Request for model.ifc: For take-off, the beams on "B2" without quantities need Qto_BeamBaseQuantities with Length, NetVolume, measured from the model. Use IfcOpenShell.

First a look at what the model holds.

```python
import ifcopenshell
import ifcopenshell.util.element
import ifcopenshell.util.unit

model = ifcopenshell.open("model.ifc")
print(model.schema)
for unit_type in ("LENGTHUNIT", "AREAUNIT", "VOLUMEUNIT"):
    print(unit_type, ifcopenshell.util.unit.calculate_unit_scale(model, unit_type))
storey = next(s for s in model.by_type("IfcBuildingStorey") if s.Name == "B2")
beams = [e for e in ifcopenshell.util.element.get_decomposition(storey) if e.is_a("IfcBeam")]
for e in sorted(beams, key=lambda e: e.id()):
    print(e.id(), e.is_a(), e.Name, list(ifcopenshell.util.element.get_psets(e, qtos_only=True)), sep=" | ")
```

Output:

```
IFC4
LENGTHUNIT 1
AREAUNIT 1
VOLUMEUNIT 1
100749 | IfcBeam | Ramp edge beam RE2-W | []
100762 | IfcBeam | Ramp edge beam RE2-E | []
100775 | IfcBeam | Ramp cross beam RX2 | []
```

```python
import ifcopenshell
import ifcopenshell.api.pset
import ifcopenshell.geom
import ifcopenshell.util.element
import ifcopenshell.util.shape
import ifcopenshell.util.unit

model = ifcopenshell.open("model.ifc")
unit_scale = ifcopenshell.util.unit.calculate_unit_scale(model)
volume_scale = ifcopenshell.util.unit.calculate_unit_scale(model, "VOLUMEUNIT")
settings = ifcopenshell.geom.settings()

storey = next(s for s in model.by_type("IfcBuildingStorey") if s.Name == "B2")
beams = [e for e in ifcopenshell.util.element.get_decomposition(storey) if e.is_a("IfcBeam")]

for e in sorted(beams, key=lambda e: e.id()):
    if ifcopenshell.util.element.get_psets(e, qtos_only=True, should_inherit=False):
        continue
    # Geometry comes back in metres, in the element's own axes.
    shape = ifcopenshell.geom.create_shape(settings, e)
    values = {
        "Length": ifcopenshell.util.shape.get_max_xyz(shape.geometry) / unit_scale,
        "NetVolume": ifcopenshell.util.shape.get_volume(shape.geometry) / volume_scale,
    }
    qto = ifcopenshell.api.pset.add_qto(model, product=e, name="Qto_BeamBaseQuantities")
    ifcopenshell.api.pset.edit_qto(model, qto=qto, properties=values)
    print(e.id(), {k: round(v, 3) for k, v in values.items()})

model.write("model_updated.ifc")
```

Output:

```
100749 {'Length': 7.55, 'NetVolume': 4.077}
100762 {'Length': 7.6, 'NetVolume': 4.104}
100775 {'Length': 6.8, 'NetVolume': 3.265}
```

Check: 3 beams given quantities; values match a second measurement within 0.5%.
